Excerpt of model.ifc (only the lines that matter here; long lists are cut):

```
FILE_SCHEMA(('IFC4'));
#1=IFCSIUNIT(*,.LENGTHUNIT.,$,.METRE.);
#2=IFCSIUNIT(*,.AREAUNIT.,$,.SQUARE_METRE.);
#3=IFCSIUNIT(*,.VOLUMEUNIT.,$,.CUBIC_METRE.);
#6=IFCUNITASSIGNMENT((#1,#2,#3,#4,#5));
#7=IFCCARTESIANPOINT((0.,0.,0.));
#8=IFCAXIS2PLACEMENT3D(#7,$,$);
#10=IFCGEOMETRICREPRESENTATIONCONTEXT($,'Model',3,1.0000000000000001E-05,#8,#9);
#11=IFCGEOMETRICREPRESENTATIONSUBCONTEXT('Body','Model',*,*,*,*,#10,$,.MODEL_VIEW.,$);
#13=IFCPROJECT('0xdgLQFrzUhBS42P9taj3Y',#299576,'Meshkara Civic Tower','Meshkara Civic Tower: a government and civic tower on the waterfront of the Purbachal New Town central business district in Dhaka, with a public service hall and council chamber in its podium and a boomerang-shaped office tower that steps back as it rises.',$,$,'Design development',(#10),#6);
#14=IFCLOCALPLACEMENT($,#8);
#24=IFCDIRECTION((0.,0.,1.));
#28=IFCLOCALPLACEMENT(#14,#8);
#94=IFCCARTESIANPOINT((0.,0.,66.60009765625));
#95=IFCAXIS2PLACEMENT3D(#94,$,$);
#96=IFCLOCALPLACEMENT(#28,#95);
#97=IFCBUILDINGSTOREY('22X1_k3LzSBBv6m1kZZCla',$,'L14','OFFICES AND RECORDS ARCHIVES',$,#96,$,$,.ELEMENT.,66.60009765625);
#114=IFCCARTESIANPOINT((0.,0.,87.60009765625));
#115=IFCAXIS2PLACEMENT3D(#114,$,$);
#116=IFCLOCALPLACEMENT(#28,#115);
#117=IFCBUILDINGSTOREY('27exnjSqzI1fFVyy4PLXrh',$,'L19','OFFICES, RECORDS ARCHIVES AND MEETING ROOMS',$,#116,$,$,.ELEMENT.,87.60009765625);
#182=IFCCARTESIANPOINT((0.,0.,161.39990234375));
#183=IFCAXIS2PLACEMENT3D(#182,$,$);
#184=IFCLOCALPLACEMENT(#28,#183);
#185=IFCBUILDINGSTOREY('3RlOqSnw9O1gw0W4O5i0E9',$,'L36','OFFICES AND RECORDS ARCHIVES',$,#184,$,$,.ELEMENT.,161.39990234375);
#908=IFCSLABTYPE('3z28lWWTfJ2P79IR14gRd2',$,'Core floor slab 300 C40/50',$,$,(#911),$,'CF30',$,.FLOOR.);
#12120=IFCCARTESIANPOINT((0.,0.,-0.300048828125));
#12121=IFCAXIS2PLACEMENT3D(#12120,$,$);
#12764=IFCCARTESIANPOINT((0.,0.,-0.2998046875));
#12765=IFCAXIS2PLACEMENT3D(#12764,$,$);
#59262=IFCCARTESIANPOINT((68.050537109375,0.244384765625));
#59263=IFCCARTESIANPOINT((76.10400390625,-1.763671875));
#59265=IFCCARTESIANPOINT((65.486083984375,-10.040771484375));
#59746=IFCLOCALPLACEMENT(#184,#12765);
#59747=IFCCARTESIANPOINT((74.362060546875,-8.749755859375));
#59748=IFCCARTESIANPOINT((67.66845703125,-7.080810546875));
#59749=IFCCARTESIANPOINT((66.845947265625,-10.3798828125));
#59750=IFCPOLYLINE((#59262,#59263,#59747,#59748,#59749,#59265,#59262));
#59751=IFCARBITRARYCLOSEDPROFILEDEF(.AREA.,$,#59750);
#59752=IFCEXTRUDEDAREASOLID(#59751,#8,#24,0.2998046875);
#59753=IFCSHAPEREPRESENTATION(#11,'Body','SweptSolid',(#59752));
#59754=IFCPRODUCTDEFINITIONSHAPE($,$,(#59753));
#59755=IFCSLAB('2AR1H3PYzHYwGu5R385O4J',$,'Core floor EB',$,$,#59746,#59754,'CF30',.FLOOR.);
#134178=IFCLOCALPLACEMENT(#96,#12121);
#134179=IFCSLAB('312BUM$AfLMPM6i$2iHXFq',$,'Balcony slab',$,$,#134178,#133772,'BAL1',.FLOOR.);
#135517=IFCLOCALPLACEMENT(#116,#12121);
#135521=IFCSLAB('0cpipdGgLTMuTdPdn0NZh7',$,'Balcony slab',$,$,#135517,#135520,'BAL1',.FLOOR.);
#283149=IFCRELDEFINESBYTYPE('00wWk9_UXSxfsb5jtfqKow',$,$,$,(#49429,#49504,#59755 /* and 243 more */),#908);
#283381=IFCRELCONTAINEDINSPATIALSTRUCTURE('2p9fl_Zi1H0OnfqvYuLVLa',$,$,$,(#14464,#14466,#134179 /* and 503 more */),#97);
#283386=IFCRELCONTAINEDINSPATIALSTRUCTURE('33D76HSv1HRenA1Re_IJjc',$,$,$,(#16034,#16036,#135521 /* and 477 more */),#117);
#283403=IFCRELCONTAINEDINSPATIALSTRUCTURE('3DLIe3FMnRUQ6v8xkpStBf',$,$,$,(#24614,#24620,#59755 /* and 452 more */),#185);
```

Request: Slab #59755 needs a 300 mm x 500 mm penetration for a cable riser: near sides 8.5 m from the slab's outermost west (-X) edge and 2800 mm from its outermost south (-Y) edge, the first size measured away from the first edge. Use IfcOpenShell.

```python
import numpy as np
import ifcopenshell
import ifcopenshell.api.feature
import ifcopenshell.api.geometry
import ifcopenshell.api.root
import ifcopenshell.geom
import ifcopenshell.util.placement
import ifcopenshell.util.representation
import ifcopenshell.util.shape
import ifcopenshell.util.unit

model = ifcopenshell.open("model.ifc")
unit_scale = ifcopenshell.util.unit.calculate_unit_scale(model)
settings = ifcopenshell.geom.settings()


def volume(element):
    """Net volume in cubic metres, openings subtracted."""
    shape = ifcopenshell.geom.create_shape(settings, element)
    return ifcopenshell.util.shape.get_volume(shape.geometry)


slab = model.by_guid("2AR1H3PYzHYwGu5R385O4J")
before = volume(slab)

# Extent in the slab's own axes, in metres. The edges named are its -X and -Y sides.
slab_shape = ifcopenshell.geom.create_shape(settings, slab)
vertices = ifcopenshell.util.shape.get_vertices(slab_shape.geometry)
x_min, y_min, bottom = vertices.min(axis=0)
top = vertices[:, 2].max()

opening = ifcopenshell.api.root.create_entity(model, ifc_class="IfcOpeningElement", name="Cable riser opening", predefined_type="OPENING")
context = ifcopenshell.util.representation.get_context(model, "Model", "Body", "MODEL_VIEW")
width, depth = 0.3, 0.5
outline = [(0.0, 0.0), (width, 0.0), (width, depth), (0.0, depth), (0.0, 0.0)]
# Overshoot both faces by 50 mm so the cut is clean.
shape = ifcopenshell.api.geometry.add_slab_representation(
    model, context=context, depth=top - bottom + 0.1, polyline=outline
)
ifcopenshell.api.geometry.assign_representation(model, product=opening, representation=shape)

matrix = ifcopenshell.util.placement.get_local_placement(slab.ObjectPlacement)
matrix[:, 3] = matrix @ np.append(np.array([x_min + 8.5, y_min + 2.8, bottom - 0.05]) / unit_scale, 1.0)
ifcopenshell.api.geometry.edit_object_placement(model, product=opening, matrix=matrix, is_si=False)
ifcopenshell.api.feature.add_feature(model, feature=opening, element=slab)

after = volume(slab)

print(f"slab volume {before:.3f} -> {after:.3f} m3")

model.write("model_updated.ifc")
```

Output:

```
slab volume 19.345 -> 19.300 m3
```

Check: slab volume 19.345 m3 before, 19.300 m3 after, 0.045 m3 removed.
